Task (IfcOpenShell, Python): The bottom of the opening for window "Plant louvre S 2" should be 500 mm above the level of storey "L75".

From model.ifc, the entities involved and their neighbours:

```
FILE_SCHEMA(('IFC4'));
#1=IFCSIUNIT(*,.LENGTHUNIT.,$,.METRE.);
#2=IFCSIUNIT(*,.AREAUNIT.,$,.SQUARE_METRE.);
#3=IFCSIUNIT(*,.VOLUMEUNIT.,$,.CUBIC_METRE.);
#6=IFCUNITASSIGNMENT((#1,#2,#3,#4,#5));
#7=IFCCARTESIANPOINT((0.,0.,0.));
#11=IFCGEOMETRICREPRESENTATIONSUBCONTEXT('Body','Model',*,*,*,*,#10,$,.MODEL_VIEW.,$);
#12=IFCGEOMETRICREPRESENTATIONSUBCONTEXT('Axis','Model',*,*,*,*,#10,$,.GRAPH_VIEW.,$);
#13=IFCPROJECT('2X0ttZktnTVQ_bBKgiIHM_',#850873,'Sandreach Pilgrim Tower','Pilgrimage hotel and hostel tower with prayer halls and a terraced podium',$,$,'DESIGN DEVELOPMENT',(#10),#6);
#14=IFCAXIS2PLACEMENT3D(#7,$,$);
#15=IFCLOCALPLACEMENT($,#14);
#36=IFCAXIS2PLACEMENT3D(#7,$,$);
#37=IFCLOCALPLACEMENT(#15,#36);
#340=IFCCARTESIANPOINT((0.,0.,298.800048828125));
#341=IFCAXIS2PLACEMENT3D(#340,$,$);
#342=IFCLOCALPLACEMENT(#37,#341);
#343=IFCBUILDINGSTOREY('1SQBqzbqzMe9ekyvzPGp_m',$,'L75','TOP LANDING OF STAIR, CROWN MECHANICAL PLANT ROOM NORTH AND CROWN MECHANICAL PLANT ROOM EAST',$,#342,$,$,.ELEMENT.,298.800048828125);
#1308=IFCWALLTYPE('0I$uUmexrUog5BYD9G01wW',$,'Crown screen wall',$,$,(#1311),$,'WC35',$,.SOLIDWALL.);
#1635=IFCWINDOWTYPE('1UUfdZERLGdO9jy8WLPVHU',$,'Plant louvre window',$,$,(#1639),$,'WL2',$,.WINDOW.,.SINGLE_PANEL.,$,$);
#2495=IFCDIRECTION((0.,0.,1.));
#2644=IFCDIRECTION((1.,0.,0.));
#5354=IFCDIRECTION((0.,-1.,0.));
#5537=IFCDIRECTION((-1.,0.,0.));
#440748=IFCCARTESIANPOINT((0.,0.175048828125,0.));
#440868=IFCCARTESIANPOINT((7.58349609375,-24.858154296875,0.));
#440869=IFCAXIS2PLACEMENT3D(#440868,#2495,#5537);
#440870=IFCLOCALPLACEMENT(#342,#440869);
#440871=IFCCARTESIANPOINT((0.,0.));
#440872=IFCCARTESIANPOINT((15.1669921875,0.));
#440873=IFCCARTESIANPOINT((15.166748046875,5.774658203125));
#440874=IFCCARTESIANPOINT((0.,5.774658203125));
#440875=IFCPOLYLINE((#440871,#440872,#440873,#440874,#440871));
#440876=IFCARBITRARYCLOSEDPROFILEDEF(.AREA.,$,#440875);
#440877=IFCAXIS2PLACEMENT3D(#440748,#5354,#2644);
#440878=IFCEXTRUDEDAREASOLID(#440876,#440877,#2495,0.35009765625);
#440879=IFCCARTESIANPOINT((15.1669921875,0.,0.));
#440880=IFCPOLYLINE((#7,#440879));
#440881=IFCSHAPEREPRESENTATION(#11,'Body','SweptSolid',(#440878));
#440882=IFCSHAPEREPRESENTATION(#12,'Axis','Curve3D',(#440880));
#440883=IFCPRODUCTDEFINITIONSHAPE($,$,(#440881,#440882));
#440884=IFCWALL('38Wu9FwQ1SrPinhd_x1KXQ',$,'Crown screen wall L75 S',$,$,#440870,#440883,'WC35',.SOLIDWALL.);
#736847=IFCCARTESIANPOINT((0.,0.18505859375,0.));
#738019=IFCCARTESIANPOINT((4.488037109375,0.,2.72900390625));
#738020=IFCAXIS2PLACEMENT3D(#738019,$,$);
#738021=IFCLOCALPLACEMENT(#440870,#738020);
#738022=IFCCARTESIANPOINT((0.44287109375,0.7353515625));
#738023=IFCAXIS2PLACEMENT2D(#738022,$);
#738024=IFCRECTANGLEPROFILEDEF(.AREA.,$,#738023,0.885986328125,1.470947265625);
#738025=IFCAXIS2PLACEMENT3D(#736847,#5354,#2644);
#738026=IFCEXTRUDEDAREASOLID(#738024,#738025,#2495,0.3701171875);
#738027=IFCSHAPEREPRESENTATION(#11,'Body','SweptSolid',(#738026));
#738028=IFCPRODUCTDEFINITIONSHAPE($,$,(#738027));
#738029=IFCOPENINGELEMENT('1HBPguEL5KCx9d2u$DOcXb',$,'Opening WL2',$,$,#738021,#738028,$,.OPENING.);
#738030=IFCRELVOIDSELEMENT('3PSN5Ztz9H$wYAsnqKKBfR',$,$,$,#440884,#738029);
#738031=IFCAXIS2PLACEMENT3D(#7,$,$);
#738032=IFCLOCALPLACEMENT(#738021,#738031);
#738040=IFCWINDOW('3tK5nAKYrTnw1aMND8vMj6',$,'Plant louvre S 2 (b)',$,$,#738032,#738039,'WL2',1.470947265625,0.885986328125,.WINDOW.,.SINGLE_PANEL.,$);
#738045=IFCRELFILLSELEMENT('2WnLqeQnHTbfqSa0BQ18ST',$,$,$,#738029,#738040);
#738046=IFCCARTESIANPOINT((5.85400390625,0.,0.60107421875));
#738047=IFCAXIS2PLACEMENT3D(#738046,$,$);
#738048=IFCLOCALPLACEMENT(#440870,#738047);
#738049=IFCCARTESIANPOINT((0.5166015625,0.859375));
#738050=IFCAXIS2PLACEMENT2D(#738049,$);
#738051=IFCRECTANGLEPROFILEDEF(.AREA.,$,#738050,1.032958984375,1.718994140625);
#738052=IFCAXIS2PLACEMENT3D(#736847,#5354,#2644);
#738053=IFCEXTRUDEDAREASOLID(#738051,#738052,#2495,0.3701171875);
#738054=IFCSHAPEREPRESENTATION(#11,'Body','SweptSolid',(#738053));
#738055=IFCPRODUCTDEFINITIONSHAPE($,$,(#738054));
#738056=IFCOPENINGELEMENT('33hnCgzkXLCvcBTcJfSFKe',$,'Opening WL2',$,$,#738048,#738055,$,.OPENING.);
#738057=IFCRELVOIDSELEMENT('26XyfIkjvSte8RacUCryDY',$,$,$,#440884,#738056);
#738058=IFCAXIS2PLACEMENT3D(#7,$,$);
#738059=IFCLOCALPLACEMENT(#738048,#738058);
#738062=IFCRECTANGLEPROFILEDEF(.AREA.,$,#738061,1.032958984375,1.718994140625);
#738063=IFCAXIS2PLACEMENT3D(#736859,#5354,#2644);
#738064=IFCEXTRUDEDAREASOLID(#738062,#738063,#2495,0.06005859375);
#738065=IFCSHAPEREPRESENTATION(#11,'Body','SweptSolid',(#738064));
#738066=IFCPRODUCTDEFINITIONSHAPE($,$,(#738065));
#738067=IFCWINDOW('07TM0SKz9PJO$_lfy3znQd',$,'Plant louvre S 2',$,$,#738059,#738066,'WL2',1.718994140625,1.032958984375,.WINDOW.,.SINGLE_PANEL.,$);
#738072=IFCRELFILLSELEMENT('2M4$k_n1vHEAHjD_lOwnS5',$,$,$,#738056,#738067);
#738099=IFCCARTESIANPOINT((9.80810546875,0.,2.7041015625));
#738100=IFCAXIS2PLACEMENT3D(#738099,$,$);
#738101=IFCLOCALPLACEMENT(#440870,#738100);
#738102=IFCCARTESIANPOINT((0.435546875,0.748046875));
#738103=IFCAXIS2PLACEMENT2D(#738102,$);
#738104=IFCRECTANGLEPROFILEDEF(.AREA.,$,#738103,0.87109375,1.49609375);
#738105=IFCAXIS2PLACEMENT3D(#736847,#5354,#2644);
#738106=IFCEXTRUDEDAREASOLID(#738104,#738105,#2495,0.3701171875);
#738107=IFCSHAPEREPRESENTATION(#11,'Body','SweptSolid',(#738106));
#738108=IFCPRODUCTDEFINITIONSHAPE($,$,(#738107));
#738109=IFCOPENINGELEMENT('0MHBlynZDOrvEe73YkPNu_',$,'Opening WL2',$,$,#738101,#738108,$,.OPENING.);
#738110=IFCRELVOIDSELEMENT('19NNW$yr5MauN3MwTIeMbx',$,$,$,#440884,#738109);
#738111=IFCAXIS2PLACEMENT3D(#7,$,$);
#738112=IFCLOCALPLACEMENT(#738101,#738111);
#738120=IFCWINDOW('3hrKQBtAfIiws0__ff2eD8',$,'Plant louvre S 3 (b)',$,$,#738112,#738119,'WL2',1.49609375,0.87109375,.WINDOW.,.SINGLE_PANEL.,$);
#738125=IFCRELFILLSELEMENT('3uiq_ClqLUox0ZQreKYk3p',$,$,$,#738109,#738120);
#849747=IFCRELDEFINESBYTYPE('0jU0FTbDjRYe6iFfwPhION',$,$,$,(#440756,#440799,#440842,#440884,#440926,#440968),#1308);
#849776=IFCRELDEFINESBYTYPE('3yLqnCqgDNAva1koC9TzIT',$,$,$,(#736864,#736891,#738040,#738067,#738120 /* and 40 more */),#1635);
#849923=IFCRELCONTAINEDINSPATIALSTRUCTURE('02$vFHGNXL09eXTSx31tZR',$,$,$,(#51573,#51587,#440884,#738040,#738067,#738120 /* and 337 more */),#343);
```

```python
import numpy as np
import ifcopenshell
import ifcopenshell.api.geometry
import ifcopenshell.geom
import ifcopenshell.util.element
import ifcopenshell.util.placement
import ifcopenshell.util.shape
import ifcopenshell.util.unit

model = ifcopenshell.open("model.ifc")
unit_scale = ifcopenshell.util.unit.calculate_unit_scale(model)

window = model.by_guid("07TM0SKz9PJO$_lfy3znQd")
opening = window.FillsVoids[0].RelatingOpeningElement
storey = ifcopenshell.util.element.get_container(window, ifc_class="IfcBuildingStorey")
level = ifcopenshell.util.placement.get_local_placement(storey.ObjectPlacement)[2, 3]

# The opening's origin need not be at the sill, so measure its lowest point.
shape = ifcopenshell.geom.create_shape(ifcopenshell.geom.settings(), opening)
bottom = ifcopenshell.util.shape.get_shape_bottom_elevation(shape, shape.geometry) / unit_scale
dz = level + 0.5 / unit_scale - bottom

shift = np.array([0.0, 0.0, dz])
# The window is placed relative to its opening, so it follows when the opening moves.
matrix = ifcopenshell.util.placement.get_local_placement(opening.ObjectPlacement)
matrix[:3, 3] += shift
ifcopenshell.api.geometry.edit_object_placement(
    model, product=opening, matrix=matrix, is_si=False, should_transform_children=True
)

print(f"moved by {dz * unit_scale:+.3f} m")

model.write("model_rev.ifc")
```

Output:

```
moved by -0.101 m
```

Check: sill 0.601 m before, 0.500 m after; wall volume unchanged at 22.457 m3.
